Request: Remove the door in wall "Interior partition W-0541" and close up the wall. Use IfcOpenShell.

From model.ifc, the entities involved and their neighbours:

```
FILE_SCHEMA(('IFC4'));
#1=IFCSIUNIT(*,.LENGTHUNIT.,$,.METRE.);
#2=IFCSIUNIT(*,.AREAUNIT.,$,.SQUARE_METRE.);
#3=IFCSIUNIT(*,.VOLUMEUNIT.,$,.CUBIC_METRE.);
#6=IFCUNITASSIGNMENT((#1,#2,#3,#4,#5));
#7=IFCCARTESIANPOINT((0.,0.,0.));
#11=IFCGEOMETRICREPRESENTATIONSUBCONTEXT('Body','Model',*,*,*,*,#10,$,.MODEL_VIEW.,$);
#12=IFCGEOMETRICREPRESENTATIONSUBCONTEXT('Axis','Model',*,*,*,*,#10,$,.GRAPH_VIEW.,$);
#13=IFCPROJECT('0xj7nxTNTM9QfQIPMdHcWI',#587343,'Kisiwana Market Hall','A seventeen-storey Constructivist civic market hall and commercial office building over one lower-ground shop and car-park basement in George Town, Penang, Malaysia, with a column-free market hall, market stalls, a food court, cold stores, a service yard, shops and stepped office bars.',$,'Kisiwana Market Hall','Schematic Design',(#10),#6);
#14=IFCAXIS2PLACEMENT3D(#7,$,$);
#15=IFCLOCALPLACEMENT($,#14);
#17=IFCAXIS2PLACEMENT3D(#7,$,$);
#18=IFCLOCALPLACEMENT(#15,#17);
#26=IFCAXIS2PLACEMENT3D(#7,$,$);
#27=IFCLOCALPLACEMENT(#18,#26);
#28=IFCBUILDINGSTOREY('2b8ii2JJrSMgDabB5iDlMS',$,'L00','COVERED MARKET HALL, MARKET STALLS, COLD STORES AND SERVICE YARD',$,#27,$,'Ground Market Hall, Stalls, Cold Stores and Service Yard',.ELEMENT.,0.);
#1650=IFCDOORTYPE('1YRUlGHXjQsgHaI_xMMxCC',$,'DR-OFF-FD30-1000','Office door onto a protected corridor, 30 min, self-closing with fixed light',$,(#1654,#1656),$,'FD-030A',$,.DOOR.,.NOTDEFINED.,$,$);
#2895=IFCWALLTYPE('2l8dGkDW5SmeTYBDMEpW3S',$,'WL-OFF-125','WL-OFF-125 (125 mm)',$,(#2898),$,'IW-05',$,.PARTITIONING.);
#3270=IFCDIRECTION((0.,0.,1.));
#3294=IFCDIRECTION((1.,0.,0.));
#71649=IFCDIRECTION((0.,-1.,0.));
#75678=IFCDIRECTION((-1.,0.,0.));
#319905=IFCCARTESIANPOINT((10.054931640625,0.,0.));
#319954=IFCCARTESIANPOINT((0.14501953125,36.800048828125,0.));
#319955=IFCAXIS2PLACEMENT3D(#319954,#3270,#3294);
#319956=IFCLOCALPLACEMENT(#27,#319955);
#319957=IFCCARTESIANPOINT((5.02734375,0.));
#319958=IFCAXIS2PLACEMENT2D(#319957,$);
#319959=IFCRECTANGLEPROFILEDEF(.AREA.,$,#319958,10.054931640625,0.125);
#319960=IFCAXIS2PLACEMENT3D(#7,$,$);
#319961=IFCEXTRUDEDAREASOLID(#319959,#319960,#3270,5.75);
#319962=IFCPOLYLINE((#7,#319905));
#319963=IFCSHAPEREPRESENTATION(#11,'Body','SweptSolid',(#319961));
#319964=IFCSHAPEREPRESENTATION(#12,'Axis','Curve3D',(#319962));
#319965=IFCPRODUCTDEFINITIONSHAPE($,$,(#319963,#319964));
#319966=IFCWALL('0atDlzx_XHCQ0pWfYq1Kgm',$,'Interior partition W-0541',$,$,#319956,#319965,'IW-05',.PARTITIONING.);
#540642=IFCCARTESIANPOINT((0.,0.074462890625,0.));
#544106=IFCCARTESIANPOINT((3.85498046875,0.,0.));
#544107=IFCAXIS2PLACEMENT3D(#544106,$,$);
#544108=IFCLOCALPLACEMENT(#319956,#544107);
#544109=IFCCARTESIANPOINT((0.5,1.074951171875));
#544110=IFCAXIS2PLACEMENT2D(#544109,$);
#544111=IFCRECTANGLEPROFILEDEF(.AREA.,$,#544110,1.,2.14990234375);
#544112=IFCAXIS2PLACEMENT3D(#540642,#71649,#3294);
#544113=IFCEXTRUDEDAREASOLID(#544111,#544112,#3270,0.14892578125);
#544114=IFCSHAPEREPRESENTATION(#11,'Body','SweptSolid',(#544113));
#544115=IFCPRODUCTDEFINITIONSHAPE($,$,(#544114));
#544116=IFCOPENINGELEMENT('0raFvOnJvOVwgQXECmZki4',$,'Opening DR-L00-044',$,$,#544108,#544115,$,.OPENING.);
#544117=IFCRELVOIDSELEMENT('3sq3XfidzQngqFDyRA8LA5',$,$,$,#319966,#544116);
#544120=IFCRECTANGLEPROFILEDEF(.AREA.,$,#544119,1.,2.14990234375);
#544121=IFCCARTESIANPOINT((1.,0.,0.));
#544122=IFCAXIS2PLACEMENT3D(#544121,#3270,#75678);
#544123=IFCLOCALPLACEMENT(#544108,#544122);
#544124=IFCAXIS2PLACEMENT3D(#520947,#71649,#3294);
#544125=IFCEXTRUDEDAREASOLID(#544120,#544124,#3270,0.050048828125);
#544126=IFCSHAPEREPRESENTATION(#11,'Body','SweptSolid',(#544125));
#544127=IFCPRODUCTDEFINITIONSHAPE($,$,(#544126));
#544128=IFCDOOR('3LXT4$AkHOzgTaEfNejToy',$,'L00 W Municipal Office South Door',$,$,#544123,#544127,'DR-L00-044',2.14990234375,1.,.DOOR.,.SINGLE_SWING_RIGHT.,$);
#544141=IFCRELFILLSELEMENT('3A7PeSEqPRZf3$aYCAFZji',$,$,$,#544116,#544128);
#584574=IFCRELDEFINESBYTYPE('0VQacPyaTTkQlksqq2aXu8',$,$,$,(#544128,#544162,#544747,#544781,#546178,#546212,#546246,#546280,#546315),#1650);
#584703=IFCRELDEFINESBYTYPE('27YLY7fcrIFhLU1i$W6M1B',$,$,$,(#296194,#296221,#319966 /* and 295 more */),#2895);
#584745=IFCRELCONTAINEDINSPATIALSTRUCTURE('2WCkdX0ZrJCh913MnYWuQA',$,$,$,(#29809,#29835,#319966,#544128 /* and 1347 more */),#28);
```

```python
import ifcopenshell
import ifcopenshell.api.feature
import ifcopenshell.api.root
import ifcopenshell.geom
import ifcopenshell.util.shape

model = ifcopenshell.open("model.ifc")
settings = ifcopenshell.geom.settings()


def volume(element):
    """Net volume in cubic metres, openings subtracted."""
    shape = ifcopenshell.geom.create_shape(settings, element)
    return ifcopenshell.util.shape.get_volume(shape.geometry)


door = model.by_id(544128)
opening = door.FillsVoids[0].RelatingOpeningElement
wall = opening.VoidsElements[0].RelatingBuildingElement
before = volume(wall)

ifcopenshell.api.root.remove_product(model, product=door)
ifcopenshell.api.feature.remove_feature(model, feature=opening)

after = volume(wall)

print(f"wall volume {before:.3f} -> {after:.3f} m3")

model.write("model-out.ifc")
```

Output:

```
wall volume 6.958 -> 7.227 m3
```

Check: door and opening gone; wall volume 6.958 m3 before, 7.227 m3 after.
